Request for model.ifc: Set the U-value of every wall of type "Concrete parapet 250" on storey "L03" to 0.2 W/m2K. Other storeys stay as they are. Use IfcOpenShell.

First a look at what the model holds.

```python
import ifcopenshell
import ifcopenshell.util.element

model = ifcopenshell.open("model.ifc")
print(model.schema)
storey = next(s for s in model.by_type("IfcBuildingStorey") if s.Name == "L03")
walls = [e for e in ifcopenshell.util.element.get_decomposition(storey) if e.is_a("IfcWall")]
seen = {}
for e in walls:
    element_type = ifcopenshell.util.element.get_type(e)
    key = (element_type.Name if element_type != e and element_type else None, ifcopenshell.util.element.get_pset(e, "Pset_WallCommon", "ThermalTransmittance"))
    seen[key] = seen.get(key, 0) + 1
for (name, value), count in sorted(seen.items(), key=str):
    print(count, "x", name, "|", value)
```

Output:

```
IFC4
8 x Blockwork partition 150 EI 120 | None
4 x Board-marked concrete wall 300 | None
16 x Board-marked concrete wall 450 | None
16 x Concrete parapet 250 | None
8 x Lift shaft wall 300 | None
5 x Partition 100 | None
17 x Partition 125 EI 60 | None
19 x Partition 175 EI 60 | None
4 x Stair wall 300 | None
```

```python
import ifcopenshell
import ifcopenshell.api.pset
import ifcopenshell.util.element

model = ifcopenshell.open("model.ifc")

storey = next(s for s in model.by_type("IfcBuildingStorey") if s.Name == "L03")
walls = [e for e in ifcopenshell.util.element.get_decomposition(storey) if e.is_a("IfcWall")]

count = 0
for e in walls:
    element_type = ifcopenshell.util.element.get_type(e)
    if element_type in (None, e) or element_type.Name != "Concrete parapet 250":
        continue
    # add_pset returns the element's existing set when there is one.
    pset = ifcopenshell.api.pset.add_pset(model, product=e, name="Pset_WallCommon")
    ifcopenshell.api.pset.edit_pset(model, pset=pset, properties={"ThermalTransmittance": 0.2})
    count += 1

print(count, "walls updated")

model.write("model_updated.ifc")
```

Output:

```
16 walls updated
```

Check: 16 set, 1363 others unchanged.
